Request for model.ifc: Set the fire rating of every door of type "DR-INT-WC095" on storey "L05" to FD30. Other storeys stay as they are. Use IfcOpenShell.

First a look at what the model holds.

```python
import ifcopenshell
import ifcopenshell.util.element

model = ifcopenshell.open("model.ifc")
print(model.schema)
storey = next(s for s in model.by_type("IfcBuildingStorey") if s.Name == "L05")
doors = [e for e in ifcopenshell.util.element.get_decomposition(storey) if e.is_a("IfcDoor")]
seen = {}
for e in doors:
    element_type = ifcopenshell.util.element.get_type(e)
    key = (element_type.Name if element_type != e and element_type else None, ifcopenshell.util.element.get_pset(e, "Pset_DoorCommon", "FireRating"))
    seen[key] = seen.get(key, 0) + 1
for (name, value), count in sorted(seen.items(), key=str):
    print(count, "x", name, "|", value)
```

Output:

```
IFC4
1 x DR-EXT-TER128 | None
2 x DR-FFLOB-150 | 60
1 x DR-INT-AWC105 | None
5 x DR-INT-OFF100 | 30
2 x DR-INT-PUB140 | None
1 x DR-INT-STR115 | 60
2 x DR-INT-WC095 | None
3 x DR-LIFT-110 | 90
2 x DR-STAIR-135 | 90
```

```python
import ifcopenshell
import ifcopenshell.api.pset
import ifcopenshell.util.element

model = ifcopenshell.open("model.ifc")

storey = next(s for s in model.by_type("IfcBuildingStorey") if s.Name == "L05")
doors = [e for e in ifcopenshell.util.element.get_decomposition(storey) if e.is_a("IfcDoor")]

count = 0
for e in doors:
    element_type = ifcopenshell.util.element.get_type(e)
    if element_type in (None, e) or element_type.Name != "DR-INT-WC095":
        continue
    # add_pset returns the element's existing set when there is one.
    pset = ifcopenshell.api.pset.add_pset(model, product=e, name="Pset_DoorCommon")
    ifcopenshell.api.pset.edit_pset(model, pset=pset, properties={"FireRating": "FD30"})
    count += 1

print(count, "doors updated")

model.write("model_updated.ifc")
```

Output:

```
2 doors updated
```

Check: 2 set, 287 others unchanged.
